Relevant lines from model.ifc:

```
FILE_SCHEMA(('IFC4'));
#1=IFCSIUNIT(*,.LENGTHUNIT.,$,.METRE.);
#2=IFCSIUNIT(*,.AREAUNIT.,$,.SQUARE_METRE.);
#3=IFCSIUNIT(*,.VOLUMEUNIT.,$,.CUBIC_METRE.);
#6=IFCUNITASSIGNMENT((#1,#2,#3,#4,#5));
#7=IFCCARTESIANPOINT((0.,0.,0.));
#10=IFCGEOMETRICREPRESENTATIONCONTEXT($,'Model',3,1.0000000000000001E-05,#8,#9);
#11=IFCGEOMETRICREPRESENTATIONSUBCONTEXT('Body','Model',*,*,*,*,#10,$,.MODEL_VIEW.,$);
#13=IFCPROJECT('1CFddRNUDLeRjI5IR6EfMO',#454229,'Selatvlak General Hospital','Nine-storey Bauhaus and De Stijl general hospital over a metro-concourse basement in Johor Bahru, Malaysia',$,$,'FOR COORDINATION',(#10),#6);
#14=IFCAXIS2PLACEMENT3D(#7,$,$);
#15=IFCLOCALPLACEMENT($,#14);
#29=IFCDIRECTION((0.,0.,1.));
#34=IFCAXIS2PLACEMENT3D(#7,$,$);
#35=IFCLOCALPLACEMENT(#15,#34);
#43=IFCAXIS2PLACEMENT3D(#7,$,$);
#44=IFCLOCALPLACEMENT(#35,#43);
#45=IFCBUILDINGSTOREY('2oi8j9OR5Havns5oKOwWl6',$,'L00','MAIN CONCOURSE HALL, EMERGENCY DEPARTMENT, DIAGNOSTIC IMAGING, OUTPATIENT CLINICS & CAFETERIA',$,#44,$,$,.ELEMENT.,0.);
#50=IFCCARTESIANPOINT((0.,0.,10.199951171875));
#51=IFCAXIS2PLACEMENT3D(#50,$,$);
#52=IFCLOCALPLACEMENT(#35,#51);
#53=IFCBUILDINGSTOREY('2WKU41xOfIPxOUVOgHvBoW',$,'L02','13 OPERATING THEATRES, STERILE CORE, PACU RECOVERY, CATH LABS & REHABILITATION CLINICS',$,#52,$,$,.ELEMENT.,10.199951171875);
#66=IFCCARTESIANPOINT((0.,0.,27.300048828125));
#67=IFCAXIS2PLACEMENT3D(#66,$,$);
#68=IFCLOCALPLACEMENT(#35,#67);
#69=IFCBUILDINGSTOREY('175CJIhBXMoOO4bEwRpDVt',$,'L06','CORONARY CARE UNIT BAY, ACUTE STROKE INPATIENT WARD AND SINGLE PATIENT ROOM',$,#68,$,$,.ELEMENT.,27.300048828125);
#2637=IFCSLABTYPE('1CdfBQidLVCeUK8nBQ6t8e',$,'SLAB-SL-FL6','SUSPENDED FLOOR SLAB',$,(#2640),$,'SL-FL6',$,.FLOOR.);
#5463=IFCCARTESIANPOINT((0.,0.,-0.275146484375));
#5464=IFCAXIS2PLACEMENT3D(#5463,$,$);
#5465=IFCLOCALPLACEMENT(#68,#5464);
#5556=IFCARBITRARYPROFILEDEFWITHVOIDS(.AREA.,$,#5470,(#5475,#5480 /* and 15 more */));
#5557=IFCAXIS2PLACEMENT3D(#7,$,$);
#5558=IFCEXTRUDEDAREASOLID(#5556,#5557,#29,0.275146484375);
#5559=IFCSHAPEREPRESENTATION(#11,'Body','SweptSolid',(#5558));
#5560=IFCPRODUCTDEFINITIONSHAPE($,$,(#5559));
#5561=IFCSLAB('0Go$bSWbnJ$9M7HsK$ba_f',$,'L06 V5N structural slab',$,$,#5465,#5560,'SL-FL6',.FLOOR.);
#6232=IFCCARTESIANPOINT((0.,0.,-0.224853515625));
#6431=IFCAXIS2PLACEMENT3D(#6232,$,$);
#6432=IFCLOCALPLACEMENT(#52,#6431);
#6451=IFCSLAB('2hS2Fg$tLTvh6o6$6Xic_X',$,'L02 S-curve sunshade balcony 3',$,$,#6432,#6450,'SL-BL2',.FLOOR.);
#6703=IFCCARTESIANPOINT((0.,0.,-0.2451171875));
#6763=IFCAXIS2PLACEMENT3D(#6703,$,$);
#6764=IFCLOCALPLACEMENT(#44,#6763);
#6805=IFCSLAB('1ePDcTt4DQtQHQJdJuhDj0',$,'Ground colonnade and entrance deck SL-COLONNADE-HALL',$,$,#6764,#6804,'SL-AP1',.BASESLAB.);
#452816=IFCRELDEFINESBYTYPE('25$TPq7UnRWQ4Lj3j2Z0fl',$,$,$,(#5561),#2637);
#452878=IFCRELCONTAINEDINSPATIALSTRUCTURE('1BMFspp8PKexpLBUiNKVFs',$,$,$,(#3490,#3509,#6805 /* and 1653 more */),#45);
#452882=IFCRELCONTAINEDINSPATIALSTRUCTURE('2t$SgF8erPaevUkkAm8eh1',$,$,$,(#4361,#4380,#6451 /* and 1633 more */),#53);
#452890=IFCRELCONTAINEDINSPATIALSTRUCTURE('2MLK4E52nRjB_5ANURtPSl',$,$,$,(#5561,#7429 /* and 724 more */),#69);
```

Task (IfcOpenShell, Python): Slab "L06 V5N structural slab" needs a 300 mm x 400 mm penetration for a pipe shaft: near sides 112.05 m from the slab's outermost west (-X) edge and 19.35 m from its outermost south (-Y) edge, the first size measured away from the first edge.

```python
import numpy as np
import ifcopenshell
import ifcopenshell.api.feature
import ifcopenshell.api.geometry
import ifcopenshell.api.root
import ifcopenshell.geom
import ifcopenshell.util.placement
import ifcopenshell.util.representation
import ifcopenshell.util.shape
import ifcopenshell.util.unit

model = ifcopenshell.open("model.ifc")
unit_scale = ifcopenshell.util.unit.calculate_unit_scale(model)
settings = ifcopenshell.geom.settings()


def volume(element):
    """Net volume in cubic metres, openings subtracted."""
    shape = ifcopenshell.geom.create_shape(settings, element)
    return ifcopenshell.util.shape.get_volume(shape.geometry)


slab = model.by_id(5561)
before = volume(slab)

# Extent in the slab's own axes, in metres. The edges named are its -X and -Y sides.
slab_shape = ifcopenshell.geom.create_shape(settings, slab)
vertices = ifcopenshell.util.shape.get_vertices(slab_shape.geometry)
x_min, y_min, bottom = vertices.min(axis=0)
top = vertices[:, 2].max()

opening = ifcopenshell.api.root.create_entity(model, ifc_class="IfcOpeningElement", name="Pipe shaft opening", predefined_type="OPENING")
context = ifcopenshell.util.representation.get_context(model, "Model", "Body", "MODEL_VIEW")
width, depth = 0.3, 0.4
outline = [(0.0, 0.0), (width, 0.0), (width, depth), (0.0, depth), (0.0, 0.0)]
# Overshoot both faces by 50 mm so the cut is clean.
shape = ifcopenshell.api.geometry.add_slab_representation(
    model, context=context, depth=top - bottom + 0.1, polyline=outline
)
ifcopenshell.api.geometry.assign_representation(model, product=opening, representation=shape)

matrix = ifcopenshell.util.placement.get_local_placement(slab.ObjectPlacement)
matrix[:, 3] = matrix @ np.append(np.array([x_min + 112.05, y_min + 19.35, bottom - 0.05]) / unit_scale, 1.0)
ifcopenshell.api.geometry.edit_object_placement(model, product=opening, matrix=matrix, is_si=False)
ifcopenshell.api.feature.add_feature(model, feature=opening, element=slab)

after = volume(slab)

print(f"slab volume {before:.3f} -> {after:.3f} m3")

model.write("model_rev.ifc")
```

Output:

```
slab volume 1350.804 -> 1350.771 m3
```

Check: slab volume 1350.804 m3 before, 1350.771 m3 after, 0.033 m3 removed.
